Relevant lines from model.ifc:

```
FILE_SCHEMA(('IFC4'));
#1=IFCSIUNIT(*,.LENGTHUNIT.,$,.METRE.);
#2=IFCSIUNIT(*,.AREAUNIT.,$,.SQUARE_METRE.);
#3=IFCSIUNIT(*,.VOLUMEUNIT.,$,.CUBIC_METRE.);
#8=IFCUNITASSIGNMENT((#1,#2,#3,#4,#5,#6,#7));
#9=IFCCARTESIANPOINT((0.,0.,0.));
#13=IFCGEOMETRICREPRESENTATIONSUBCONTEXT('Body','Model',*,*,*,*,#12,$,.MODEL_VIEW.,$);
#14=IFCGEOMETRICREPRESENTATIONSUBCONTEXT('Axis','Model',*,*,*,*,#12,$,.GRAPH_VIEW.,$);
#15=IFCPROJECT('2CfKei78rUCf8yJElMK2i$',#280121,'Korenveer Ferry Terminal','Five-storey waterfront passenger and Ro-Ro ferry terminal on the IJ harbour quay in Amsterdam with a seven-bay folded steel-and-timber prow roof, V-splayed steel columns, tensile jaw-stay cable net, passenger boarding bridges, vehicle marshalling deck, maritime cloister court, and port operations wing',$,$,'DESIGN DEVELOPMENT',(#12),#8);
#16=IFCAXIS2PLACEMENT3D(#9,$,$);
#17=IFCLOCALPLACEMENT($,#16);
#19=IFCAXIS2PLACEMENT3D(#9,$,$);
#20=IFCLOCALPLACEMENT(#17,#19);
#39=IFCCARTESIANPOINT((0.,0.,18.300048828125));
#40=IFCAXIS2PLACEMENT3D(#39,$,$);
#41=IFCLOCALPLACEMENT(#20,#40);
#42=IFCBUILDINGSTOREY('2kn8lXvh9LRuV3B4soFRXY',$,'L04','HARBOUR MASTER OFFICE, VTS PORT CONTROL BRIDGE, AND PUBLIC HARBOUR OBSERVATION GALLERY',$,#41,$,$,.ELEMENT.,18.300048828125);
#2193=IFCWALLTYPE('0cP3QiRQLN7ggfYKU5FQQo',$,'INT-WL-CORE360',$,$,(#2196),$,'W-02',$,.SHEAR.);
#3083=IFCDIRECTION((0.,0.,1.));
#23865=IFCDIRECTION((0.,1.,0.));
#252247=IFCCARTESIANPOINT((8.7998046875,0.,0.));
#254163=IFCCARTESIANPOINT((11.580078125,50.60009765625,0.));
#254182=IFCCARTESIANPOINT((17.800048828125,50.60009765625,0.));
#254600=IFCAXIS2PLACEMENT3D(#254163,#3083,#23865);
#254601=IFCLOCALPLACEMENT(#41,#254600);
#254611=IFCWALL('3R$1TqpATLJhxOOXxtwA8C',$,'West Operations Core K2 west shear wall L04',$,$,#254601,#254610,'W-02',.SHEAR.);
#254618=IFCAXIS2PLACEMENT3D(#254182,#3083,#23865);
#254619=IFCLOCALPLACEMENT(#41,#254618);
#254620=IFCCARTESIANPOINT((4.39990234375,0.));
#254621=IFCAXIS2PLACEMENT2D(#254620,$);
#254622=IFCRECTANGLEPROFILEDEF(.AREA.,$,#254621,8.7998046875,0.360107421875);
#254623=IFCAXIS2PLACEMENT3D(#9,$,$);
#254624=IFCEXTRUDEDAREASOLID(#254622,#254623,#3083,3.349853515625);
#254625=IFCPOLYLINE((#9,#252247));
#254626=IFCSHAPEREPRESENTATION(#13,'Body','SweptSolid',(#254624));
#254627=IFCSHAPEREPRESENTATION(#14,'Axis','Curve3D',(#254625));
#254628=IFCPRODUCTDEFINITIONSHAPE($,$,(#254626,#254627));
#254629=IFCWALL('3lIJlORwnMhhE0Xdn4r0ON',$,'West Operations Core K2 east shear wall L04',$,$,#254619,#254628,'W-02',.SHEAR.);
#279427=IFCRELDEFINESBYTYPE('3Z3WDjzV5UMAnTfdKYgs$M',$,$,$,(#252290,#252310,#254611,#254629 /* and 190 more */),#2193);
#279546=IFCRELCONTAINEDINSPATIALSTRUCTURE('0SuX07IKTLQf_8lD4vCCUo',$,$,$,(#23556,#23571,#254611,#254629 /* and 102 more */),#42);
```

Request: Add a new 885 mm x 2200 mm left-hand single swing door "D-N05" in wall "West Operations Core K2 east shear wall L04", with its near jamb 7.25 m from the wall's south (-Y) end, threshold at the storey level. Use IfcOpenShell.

```python
import numpy as np
import ifcopenshell
import ifcopenshell.api.feature
import ifcopenshell.api.geometry
import ifcopenshell.api.root
import ifcopenshell.api.spatial
import ifcopenshell.geom
import ifcopenshell.util.element
import ifcopenshell.util.placement
import ifcopenshell.util.representation
import ifcopenshell.util.shape
import ifcopenshell.util.unit

model = ifcopenshell.open("model.ifc")
unit_scale = ifcopenshell.util.unit.calculate_unit_scale(model)
settings = ifcopenshell.geom.settings()


def volume(element):
    """Net volume in cubic metres, openings subtracted."""
    shape = ifcopenshell.geom.create_shape(settings, element)
    return ifcopenshell.util.shape.get_volume(shape.geometry)


wall = model.by_id(254629)
storey = ifcopenshell.util.element.get_container(wall, ifc_class="IfcBuildingStorey")
context = ifcopenshell.util.representation.get_context(model, "Model", "Body", "MODEL_VIEW")
before = volume(wall)

width, height, from_end, sill = 0.885, 2.2, 7.25, 0.0  # metres

# The wall runs along its own X axis, and the end named is its -X end.
wall_shape = ifcopenshell.geom.create_shape(settings, wall)
x, y, z = ifcopenshell.util.shape.get_vertices(wall_shape.geometry).T
start = x.min() + from_end
face, thickness = float(y.min()), float(y.max() - y.min())
wall_matrix = ifcopenshell.util.placement.get_local_placement(wall.ObjectPlacement)
level = ifcopenshell.util.placement.get_local_placement(storey.ObjectPlacement)[2, 3]


def in_wall(x, y):
    """Placement at x, y metres in the wall's axes, at sill height."""
    matrix = wall_matrix.copy()
    matrix[:, 3] = wall_matrix @ np.array([x / unit_scale, y / unit_scale, 0.0, 1.0])
    matrix[2, 3] = level + sill / unit_scale
    return matrix


# Opening: a box that overshoots both wall faces by 50 mm.
opening = ifcopenshell.api.root.create_entity(model, ifc_class="IfcOpeningElement", predefined_type="OPENING")
box = ifcopenshell.api.geometry.add_wall_representation(
    model, context=context, length=width, height=height, thickness=thickness + 0.1
)
ifcopenshell.api.geometry.assign_representation(model, product=opening, representation=box)
ifcopenshell.api.geometry.edit_object_placement(model, product=opening, matrix=in_wall(start, face - 0.05), is_si=False)
ifcopenshell.api.feature.add_feature(model, feature=opening, element=wall)

door = ifcopenshell.api.root.create_entity(model, ifc_class="IfcDoor", name="D-N05", predefined_type="DOOR")
door.OverallWidth, door.OverallHeight = width / unit_scale, height / unit_scale
door.OperationType = "SINGLE_SWING_LEFT"
body = ifcopenshell.api.geometry.add_door_representation(
    model,
    context=context,
    overall_width=door.OverallWidth,
    overall_height=door.OverallHeight,
    operation_type="SINGLE_SWING_LEFT",
    lining_properties={"LiningDepth": thickness / unit_scale, "ThresholdDepth": thickness / unit_scale},
)
ifcopenshell.api.geometry.assign_representation(model, product=door, representation=body)
ifcopenshell.api.spatial.assign_container(model, products=[door], relating_structure=storey)
ifcopenshell.api.feature.add_filling(model, opening=opening, element=door)

# The lining spans the wall, so the door starts at the wall face.
ifcopenshell.api.geometry.edit_object_placement(model, product=door, matrix=in_wall(start, face), is_si=False)

after = volume(wall)

print(f"wall volume {before:.3f} -> {after:.3f} m3")

model.write("model_updated.ifc")
```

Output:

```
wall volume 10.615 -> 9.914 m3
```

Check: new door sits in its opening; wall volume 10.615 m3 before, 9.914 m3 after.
